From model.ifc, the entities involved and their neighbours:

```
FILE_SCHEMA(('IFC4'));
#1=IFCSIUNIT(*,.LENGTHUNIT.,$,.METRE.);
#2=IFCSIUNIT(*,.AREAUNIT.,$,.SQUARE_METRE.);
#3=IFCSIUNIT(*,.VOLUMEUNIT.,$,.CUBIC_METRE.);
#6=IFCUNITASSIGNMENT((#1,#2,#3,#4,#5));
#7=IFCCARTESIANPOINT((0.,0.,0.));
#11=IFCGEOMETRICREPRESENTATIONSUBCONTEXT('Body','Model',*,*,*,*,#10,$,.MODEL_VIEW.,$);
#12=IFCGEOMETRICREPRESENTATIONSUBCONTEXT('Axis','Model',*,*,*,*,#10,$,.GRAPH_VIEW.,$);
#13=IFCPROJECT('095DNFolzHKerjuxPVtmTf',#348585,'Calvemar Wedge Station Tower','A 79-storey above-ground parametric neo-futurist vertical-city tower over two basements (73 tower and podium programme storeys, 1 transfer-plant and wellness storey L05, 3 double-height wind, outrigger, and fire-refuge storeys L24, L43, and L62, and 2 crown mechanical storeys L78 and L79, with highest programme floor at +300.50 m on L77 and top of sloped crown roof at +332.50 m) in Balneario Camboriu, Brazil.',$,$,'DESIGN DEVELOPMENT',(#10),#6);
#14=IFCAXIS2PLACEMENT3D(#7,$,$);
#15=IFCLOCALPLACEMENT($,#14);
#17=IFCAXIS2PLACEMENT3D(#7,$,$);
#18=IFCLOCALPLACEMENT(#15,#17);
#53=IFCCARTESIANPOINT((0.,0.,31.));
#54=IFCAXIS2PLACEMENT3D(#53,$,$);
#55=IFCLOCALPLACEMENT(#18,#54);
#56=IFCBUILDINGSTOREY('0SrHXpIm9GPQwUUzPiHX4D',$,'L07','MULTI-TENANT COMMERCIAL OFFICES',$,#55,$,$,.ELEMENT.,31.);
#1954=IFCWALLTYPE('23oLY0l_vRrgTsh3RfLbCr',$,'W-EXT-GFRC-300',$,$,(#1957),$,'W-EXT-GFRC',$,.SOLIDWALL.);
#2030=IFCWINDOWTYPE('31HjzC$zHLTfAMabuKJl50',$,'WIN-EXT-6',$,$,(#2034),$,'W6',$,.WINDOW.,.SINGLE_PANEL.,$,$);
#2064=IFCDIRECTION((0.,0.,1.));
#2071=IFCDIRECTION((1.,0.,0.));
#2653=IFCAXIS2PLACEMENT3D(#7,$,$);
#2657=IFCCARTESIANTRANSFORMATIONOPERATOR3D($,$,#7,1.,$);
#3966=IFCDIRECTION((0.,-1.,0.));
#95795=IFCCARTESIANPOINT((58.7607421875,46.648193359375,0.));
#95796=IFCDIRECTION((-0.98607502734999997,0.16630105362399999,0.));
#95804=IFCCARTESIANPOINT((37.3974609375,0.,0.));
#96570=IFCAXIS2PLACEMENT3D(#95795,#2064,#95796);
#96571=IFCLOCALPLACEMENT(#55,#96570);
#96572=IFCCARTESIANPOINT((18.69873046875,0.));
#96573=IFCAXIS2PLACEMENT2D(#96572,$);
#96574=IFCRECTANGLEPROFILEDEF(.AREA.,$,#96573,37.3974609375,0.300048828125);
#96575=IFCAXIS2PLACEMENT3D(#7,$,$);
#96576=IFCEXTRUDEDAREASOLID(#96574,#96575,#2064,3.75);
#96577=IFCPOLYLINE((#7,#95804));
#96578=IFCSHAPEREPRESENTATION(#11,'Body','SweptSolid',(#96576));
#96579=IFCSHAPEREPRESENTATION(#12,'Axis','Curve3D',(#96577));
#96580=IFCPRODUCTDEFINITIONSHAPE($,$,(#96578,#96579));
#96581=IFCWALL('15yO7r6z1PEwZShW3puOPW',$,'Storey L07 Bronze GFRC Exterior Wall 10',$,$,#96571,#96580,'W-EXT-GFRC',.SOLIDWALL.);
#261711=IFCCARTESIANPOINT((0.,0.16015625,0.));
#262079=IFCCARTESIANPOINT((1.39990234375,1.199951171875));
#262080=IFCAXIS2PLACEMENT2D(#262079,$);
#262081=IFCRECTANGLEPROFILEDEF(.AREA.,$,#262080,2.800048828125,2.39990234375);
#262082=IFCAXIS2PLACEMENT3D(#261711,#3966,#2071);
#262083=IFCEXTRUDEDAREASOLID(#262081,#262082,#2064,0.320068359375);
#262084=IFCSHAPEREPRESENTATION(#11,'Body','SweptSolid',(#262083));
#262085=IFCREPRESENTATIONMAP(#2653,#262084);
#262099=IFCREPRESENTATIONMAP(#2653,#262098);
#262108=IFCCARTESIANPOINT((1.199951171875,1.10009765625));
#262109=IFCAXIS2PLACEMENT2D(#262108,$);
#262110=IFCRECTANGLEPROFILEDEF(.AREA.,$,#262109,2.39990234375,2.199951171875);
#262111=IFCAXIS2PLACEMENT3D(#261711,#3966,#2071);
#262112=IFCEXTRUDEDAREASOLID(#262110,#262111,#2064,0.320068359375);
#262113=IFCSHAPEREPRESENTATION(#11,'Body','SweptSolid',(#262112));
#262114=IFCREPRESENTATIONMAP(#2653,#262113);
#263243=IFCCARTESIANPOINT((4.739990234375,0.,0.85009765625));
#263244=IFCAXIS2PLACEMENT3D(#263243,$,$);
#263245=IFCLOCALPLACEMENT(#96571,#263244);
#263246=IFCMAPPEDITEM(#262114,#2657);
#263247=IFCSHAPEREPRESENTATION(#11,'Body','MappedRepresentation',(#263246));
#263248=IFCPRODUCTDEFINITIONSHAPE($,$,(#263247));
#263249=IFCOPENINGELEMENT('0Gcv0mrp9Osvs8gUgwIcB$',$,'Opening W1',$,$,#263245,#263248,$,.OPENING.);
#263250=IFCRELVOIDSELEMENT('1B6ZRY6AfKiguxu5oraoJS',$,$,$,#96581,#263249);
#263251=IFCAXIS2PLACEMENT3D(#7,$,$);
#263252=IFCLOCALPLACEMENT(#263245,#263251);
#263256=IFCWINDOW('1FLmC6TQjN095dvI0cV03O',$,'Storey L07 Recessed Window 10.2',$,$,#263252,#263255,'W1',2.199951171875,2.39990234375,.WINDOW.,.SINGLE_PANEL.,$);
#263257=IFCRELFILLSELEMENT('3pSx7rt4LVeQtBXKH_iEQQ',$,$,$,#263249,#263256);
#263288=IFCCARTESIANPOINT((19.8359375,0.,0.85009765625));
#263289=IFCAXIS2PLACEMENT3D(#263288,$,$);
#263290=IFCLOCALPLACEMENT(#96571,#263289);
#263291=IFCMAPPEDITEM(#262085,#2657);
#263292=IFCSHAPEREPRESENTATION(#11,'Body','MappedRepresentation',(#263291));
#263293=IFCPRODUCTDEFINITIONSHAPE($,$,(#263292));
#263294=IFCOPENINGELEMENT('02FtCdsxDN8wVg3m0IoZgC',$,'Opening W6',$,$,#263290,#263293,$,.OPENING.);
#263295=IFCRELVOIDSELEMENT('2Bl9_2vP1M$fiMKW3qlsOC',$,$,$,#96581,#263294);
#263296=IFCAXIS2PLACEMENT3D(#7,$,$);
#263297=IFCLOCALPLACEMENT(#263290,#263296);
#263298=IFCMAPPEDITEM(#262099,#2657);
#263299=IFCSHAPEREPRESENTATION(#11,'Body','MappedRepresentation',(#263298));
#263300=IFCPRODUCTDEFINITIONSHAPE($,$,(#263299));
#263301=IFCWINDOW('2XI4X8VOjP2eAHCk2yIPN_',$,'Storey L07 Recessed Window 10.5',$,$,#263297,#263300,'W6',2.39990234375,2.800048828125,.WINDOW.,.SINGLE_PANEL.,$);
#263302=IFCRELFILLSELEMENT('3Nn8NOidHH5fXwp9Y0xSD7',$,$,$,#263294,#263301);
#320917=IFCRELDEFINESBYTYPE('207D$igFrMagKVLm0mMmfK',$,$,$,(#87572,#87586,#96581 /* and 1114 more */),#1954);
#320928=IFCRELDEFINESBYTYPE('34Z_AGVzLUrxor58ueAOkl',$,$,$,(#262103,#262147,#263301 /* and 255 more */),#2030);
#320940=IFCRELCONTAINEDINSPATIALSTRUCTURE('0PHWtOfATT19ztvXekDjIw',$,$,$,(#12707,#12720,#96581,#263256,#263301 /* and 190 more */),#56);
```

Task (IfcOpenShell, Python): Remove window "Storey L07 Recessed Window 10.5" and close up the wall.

```python
import ifcopenshell
import ifcopenshell.api.feature
import ifcopenshell.api.root
import ifcopenshell.geom
import ifcopenshell.util.shape

model = ifcopenshell.open("model.ifc")
settings = ifcopenshell.geom.settings()


def volume(element):
    """Net volume in cubic metres, openings subtracted."""
    shape = ifcopenshell.geom.create_shape(settings, element)
    return ifcopenshell.util.shape.get_volume(shape.geometry)


window = model.by_guid("2XI4X8VOjP2eAHCk2yIPN_")
opening = window.FillsVoids[0].RelatingOpeningElement
wall = opening.VoidsElements[0].RelatingBuildingElement
before = volume(wall)

ifcopenshell.api.root.remove_product(model, product=window)
ifcopenshell.api.feature.remove_feature(model, feature=opening)

after = volume(wall)

print(f"wall volume {before:.3f} -> {after:.3f} m3")

model.write("model_edited.ifc")
```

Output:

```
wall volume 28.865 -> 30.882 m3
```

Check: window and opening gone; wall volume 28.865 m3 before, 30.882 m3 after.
